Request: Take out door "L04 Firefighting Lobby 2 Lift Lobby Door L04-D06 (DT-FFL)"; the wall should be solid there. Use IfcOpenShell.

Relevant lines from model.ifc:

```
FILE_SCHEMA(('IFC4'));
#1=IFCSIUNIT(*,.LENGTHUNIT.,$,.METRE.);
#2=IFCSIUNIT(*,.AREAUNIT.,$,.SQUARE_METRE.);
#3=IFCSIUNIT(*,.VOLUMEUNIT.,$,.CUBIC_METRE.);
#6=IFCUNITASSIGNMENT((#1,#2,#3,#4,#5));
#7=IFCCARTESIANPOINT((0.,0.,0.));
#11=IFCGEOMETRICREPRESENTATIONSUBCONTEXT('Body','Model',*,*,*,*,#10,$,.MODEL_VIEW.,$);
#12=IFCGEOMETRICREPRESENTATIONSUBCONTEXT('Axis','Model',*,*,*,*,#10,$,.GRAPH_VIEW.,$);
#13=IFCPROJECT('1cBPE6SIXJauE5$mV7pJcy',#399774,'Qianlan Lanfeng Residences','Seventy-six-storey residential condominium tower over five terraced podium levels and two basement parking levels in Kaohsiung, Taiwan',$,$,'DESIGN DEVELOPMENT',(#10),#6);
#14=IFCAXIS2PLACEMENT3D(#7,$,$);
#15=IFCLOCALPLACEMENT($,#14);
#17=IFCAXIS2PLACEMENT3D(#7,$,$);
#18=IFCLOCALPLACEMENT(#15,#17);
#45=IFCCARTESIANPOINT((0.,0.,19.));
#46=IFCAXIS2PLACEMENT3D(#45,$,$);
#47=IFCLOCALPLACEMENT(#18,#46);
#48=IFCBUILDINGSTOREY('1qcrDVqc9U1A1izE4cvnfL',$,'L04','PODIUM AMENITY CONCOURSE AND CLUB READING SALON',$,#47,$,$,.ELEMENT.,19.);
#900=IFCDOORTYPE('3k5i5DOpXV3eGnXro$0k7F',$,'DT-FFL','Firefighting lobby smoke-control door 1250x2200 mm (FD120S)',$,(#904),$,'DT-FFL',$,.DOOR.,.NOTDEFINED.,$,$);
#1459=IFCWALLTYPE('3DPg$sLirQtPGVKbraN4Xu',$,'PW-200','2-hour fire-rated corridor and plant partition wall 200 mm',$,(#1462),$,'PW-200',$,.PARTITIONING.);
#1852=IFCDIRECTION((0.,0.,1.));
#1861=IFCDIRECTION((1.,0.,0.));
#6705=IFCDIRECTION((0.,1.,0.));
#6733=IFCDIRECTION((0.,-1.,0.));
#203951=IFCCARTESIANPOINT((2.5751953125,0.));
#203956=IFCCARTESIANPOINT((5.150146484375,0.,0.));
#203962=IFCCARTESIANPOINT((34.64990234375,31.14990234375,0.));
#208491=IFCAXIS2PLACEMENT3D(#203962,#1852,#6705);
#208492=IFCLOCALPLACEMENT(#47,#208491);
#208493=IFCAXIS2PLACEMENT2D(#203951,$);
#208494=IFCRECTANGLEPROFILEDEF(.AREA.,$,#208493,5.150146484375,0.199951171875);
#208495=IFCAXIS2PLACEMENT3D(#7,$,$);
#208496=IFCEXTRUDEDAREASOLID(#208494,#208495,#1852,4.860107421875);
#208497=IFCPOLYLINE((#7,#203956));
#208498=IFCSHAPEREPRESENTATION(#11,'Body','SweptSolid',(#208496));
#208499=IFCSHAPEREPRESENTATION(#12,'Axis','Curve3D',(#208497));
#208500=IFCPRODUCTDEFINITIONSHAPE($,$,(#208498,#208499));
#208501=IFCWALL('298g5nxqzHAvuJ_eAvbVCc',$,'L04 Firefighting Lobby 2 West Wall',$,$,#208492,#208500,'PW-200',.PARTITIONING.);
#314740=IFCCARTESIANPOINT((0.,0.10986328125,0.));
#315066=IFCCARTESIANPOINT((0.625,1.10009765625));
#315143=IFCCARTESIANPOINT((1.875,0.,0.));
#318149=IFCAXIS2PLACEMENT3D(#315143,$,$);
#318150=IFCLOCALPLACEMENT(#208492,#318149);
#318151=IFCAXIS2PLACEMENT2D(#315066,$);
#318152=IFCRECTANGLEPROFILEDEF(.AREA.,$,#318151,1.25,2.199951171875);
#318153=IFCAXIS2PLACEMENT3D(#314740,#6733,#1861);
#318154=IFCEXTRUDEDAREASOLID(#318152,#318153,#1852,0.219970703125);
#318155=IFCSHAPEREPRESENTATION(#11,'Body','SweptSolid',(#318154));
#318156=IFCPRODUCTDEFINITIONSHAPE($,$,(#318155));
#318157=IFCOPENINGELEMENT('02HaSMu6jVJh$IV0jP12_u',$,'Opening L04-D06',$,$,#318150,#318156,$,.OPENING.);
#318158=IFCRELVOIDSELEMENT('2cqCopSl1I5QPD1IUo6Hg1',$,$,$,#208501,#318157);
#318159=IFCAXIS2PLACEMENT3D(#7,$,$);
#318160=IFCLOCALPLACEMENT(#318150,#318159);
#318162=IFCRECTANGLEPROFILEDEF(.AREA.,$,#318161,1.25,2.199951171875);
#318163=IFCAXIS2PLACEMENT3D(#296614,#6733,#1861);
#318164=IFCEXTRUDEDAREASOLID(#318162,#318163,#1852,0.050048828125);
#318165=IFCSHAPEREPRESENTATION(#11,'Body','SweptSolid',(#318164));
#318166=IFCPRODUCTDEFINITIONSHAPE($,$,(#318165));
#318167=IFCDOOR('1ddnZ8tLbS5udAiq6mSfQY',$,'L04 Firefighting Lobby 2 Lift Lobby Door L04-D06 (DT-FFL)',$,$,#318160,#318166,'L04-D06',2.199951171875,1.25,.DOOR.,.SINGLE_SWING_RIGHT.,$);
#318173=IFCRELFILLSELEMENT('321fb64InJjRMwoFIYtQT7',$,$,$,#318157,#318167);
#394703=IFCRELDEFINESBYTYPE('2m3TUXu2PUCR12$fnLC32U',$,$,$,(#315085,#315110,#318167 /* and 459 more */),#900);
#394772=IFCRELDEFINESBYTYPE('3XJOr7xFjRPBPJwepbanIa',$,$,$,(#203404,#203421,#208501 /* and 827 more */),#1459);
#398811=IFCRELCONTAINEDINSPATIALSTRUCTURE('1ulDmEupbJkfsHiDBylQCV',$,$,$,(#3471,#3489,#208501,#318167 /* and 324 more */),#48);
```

```python
import ifcopenshell
import ifcopenshell.api.feature
import ifcopenshell.api.root
import ifcopenshell.geom
import ifcopenshell.util.shape

model = ifcopenshell.open("model.ifc")
settings = ifcopenshell.geom.settings()


def volume(element):
    """Net volume in cubic metres, openings subtracted."""
    shape = ifcopenshell.geom.create_shape(settings, element)
    return ifcopenshell.util.shape.get_volume(shape.geometry)


door = model.by_id(318167)
opening = door.FillsVoids[0].RelatingOpeningElement
wall = opening.VoidsElements[0].RelatingBuildingElement
before = volume(wall)

ifcopenshell.api.root.remove_product(model, product=door)
ifcopenshell.api.feature.remove_feature(model, feature=opening)

after = volume(wall)

print(f"wall volume {before:.3f} -> {after:.3f} m3")

model.write("model_v2.ifc")
```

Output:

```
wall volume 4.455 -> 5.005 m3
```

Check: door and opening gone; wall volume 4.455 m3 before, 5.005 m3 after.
